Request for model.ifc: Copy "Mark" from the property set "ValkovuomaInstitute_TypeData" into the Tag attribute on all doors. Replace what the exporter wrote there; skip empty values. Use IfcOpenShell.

First a look at what the model holds.

```python
import ifcopenshell
import ifcopenshell.util.element

model = ifcopenshell.open("model.ifc")
print(model.schema)
doors = model.by_type("IfcDoor")
print(len(doors), "doors")
for e in doors[:8]:
    source = ifcopenshell.util.element.get_pset(e, "ValkovuomaInstitute_TypeData", "Mark")
    target = e.Tag
    print(e.id(), repr(source), repr(target), sep=" | ")
```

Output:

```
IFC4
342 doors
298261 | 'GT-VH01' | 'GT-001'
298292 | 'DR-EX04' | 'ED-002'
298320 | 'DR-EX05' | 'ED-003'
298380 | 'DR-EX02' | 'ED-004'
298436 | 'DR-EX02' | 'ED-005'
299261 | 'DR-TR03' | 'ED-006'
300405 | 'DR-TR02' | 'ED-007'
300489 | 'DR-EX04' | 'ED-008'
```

```python
import ifcopenshell
import ifcopenshell.util.element

model = ifcopenshell.open("model.ifc")

count = 0
for e in model.by_type("IfcDoor"):
    value = ifcopenshell.util.element.get_pset(e, "ValkovuomaInstitute_TypeData", "Mark")
    current = e.Tag
    if not value or not value.strip() or current == value:
        continue
    e.Tag = value
    count += 1

print(count, "doors updated")

model.write("model_updated.ifc")
```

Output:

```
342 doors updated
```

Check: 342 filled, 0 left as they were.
